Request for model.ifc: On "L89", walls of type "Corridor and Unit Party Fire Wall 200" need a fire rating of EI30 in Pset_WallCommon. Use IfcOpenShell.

First a look at what the model holds.

```python
import ifcopenshell
import ifcopenshell.util.element

model = ifcopenshell.open("model.ifc")
print(model.schema)
storey = next(s for s in model.by_type("IfcBuildingStorey") if s.Name == "L89")
walls = [e for e in ifcopenshell.util.element.get_decomposition(storey) if e.is_a("IfcWall")]
seen = {}
for e in walls:
    element_type = ifcopenshell.util.element.get_type(e)
    key = (element_type.Name if element_type != e and element_type else None, ifcopenshell.util.element.get_pset(e, "Pset_WallCommon", "FireRating"))
    seen[key] = seen.get(key, 0) + 1
for (name, value), count in sorted(seen.items(), key=str):
    print(count, "x", name, "|", value)
```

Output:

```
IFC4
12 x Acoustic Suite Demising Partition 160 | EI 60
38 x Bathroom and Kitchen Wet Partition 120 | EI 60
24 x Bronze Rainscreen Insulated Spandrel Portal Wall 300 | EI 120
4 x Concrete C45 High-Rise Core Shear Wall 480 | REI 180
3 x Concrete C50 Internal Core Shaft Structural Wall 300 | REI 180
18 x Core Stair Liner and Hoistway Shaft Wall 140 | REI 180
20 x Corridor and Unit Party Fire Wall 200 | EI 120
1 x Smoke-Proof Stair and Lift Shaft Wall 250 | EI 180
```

```python
import ifcopenshell
import ifcopenshell.api.pset
import ifcopenshell.util.element

model = ifcopenshell.open("model.ifc")

storey = next(s for s in model.by_type("IfcBuildingStorey") if s.Name == "L89")
walls = [e for e in ifcopenshell.util.element.get_decomposition(storey) if e.is_a("IfcWall")]

count = 0
for e in walls:
    element_type = ifcopenshell.util.element.get_type(e)
    if element_type in (None, e) or element_type.Name != "Corridor and Unit Party Fire Wall 200":
        continue
    found = ifcopenshell.util.element.get_pset(e, "Pset_WallCommon", should_inherit=False)
    if found:
        pset = model.by_id(found["id"])
        if len(ifcopenshell.util.element.get_elements_by_pset(pset)) > 1:
            pset = ifcopenshell.api.pset.unshare_pset(model, products=[e], pset=pset)[0]
    else:
        pset = ifcopenshell.api.pset.add_pset(model, product=e, name="Pset_WallCommon")
    ifcopenshell.api.pset.edit_pset(model, pset=pset, properties={"FireRating": "EI30"})
    count += 1

print(count, "walls updated")

model.write("model_v2.ifc")
```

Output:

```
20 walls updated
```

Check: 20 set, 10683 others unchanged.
